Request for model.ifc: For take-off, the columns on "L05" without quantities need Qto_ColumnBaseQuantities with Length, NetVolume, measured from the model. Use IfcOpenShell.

First a look at what the model holds.

```python
import ifcopenshell
import ifcopenshell.util.element
import ifcopenshell.util.unit

model = ifcopenshell.open("model.ifc")
print(model.schema)
for unit_type in ("LENGTHUNIT", "AREAUNIT", "VOLUMEUNIT"):
    print(unit_type, ifcopenshell.util.unit.calculate_unit_scale(model, unit_type))
storey = next(s for s in model.by_type("IfcBuildingStorey") if s.Name == "L05")
columns = [e for e in ifcopenshell.util.element.get_decomposition(storey) if e.is_a("IfcColumn")]
for e in sorted(columns, key=lambda e: e.id()):
    print(e.id(), e.is_a(), e.Name, list(ifcopenshell.util.element.get_psets(e, qtos_only=True)), sep=" | ")
```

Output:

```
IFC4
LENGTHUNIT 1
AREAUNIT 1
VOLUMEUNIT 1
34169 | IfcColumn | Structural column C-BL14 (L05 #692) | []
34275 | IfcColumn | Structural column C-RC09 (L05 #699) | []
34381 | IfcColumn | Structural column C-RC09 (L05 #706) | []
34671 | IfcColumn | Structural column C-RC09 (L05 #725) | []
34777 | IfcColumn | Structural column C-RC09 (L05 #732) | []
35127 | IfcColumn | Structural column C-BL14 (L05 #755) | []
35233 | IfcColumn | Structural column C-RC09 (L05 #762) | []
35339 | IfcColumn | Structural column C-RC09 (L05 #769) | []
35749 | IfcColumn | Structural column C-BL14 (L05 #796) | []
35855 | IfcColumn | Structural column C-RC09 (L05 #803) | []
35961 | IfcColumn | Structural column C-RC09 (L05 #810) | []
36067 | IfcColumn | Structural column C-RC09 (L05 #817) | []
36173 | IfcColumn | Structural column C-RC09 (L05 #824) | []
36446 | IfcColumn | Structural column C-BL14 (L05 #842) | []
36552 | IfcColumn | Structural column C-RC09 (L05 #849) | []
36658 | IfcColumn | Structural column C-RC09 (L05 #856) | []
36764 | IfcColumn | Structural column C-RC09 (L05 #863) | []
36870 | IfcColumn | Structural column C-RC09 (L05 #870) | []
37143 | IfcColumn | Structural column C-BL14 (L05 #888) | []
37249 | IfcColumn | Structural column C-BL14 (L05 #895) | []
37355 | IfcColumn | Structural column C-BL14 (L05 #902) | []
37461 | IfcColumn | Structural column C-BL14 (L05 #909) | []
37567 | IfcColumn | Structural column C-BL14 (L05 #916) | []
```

```python
import ifcopenshell
import ifcopenshell.api.pset
import ifcopenshell.geom
import ifcopenshell.util.element
import ifcopenshell.util.shape
import ifcopenshell.util.unit

model = ifcopenshell.open("model.ifc")
unit_scale = ifcopenshell.util.unit.calculate_unit_scale(model)
volume_scale = ifcopenshell.util.unit.calculate_unit_scale(model, "VOLUMEUNIT")
settings = ifcopenshell.geom.settings()

storey = next(s for s in model.by_type("IfcBuildingStorey") if s.Name == "L05")
columns = [e for e in ifcopenshell.util.element.get_decomposition(storey) if e.is_a("IfcColumn")]

for e in sorted(columns, key=lambda e: e.id()):
    if ifcopenshell.util.element.get_psets(e, qtos_only=True, should_inherit=False):
        continue
    # Geometry comes back in metres, in the element's own axes.
    shape = ifcopenshell.geom.create_shape(settings, e)
    values = {
        "Length": ifcopenshell.util.shape.get_z(shape.geometry) / unit_scale,
        "NetVolume": ifcopenshell.util.shape.get_volume(shape.geometry) / volume_scale,
    }
    qto = ifcopenshell.api.pset.add_qto(model, product=e, name="Qto_ColumnBaseQuantities")
    ifcopenshell.api.pset.edit_qto(model, qto=qto, properties=values)
    print(e.id(), {k: round(v, 3) for k, v in values.items()})

model.write("model_edited.ifc")
```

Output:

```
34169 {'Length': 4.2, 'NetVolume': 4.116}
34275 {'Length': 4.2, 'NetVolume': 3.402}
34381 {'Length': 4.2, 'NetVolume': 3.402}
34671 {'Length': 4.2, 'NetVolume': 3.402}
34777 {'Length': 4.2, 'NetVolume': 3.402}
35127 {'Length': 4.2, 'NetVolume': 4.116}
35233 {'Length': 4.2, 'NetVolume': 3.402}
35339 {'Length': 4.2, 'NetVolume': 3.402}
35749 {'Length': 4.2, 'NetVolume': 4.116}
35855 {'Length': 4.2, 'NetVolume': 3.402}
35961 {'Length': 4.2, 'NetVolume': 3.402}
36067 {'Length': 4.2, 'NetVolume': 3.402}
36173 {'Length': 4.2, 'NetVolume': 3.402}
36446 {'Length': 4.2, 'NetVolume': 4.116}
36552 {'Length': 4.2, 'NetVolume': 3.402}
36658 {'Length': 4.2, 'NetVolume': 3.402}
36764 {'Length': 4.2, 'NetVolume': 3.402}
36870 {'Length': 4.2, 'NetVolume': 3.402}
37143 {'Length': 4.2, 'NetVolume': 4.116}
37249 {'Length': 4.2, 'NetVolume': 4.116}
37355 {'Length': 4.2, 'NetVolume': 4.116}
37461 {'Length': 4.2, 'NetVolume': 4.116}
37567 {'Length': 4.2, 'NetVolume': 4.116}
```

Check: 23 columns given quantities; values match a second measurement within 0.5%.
